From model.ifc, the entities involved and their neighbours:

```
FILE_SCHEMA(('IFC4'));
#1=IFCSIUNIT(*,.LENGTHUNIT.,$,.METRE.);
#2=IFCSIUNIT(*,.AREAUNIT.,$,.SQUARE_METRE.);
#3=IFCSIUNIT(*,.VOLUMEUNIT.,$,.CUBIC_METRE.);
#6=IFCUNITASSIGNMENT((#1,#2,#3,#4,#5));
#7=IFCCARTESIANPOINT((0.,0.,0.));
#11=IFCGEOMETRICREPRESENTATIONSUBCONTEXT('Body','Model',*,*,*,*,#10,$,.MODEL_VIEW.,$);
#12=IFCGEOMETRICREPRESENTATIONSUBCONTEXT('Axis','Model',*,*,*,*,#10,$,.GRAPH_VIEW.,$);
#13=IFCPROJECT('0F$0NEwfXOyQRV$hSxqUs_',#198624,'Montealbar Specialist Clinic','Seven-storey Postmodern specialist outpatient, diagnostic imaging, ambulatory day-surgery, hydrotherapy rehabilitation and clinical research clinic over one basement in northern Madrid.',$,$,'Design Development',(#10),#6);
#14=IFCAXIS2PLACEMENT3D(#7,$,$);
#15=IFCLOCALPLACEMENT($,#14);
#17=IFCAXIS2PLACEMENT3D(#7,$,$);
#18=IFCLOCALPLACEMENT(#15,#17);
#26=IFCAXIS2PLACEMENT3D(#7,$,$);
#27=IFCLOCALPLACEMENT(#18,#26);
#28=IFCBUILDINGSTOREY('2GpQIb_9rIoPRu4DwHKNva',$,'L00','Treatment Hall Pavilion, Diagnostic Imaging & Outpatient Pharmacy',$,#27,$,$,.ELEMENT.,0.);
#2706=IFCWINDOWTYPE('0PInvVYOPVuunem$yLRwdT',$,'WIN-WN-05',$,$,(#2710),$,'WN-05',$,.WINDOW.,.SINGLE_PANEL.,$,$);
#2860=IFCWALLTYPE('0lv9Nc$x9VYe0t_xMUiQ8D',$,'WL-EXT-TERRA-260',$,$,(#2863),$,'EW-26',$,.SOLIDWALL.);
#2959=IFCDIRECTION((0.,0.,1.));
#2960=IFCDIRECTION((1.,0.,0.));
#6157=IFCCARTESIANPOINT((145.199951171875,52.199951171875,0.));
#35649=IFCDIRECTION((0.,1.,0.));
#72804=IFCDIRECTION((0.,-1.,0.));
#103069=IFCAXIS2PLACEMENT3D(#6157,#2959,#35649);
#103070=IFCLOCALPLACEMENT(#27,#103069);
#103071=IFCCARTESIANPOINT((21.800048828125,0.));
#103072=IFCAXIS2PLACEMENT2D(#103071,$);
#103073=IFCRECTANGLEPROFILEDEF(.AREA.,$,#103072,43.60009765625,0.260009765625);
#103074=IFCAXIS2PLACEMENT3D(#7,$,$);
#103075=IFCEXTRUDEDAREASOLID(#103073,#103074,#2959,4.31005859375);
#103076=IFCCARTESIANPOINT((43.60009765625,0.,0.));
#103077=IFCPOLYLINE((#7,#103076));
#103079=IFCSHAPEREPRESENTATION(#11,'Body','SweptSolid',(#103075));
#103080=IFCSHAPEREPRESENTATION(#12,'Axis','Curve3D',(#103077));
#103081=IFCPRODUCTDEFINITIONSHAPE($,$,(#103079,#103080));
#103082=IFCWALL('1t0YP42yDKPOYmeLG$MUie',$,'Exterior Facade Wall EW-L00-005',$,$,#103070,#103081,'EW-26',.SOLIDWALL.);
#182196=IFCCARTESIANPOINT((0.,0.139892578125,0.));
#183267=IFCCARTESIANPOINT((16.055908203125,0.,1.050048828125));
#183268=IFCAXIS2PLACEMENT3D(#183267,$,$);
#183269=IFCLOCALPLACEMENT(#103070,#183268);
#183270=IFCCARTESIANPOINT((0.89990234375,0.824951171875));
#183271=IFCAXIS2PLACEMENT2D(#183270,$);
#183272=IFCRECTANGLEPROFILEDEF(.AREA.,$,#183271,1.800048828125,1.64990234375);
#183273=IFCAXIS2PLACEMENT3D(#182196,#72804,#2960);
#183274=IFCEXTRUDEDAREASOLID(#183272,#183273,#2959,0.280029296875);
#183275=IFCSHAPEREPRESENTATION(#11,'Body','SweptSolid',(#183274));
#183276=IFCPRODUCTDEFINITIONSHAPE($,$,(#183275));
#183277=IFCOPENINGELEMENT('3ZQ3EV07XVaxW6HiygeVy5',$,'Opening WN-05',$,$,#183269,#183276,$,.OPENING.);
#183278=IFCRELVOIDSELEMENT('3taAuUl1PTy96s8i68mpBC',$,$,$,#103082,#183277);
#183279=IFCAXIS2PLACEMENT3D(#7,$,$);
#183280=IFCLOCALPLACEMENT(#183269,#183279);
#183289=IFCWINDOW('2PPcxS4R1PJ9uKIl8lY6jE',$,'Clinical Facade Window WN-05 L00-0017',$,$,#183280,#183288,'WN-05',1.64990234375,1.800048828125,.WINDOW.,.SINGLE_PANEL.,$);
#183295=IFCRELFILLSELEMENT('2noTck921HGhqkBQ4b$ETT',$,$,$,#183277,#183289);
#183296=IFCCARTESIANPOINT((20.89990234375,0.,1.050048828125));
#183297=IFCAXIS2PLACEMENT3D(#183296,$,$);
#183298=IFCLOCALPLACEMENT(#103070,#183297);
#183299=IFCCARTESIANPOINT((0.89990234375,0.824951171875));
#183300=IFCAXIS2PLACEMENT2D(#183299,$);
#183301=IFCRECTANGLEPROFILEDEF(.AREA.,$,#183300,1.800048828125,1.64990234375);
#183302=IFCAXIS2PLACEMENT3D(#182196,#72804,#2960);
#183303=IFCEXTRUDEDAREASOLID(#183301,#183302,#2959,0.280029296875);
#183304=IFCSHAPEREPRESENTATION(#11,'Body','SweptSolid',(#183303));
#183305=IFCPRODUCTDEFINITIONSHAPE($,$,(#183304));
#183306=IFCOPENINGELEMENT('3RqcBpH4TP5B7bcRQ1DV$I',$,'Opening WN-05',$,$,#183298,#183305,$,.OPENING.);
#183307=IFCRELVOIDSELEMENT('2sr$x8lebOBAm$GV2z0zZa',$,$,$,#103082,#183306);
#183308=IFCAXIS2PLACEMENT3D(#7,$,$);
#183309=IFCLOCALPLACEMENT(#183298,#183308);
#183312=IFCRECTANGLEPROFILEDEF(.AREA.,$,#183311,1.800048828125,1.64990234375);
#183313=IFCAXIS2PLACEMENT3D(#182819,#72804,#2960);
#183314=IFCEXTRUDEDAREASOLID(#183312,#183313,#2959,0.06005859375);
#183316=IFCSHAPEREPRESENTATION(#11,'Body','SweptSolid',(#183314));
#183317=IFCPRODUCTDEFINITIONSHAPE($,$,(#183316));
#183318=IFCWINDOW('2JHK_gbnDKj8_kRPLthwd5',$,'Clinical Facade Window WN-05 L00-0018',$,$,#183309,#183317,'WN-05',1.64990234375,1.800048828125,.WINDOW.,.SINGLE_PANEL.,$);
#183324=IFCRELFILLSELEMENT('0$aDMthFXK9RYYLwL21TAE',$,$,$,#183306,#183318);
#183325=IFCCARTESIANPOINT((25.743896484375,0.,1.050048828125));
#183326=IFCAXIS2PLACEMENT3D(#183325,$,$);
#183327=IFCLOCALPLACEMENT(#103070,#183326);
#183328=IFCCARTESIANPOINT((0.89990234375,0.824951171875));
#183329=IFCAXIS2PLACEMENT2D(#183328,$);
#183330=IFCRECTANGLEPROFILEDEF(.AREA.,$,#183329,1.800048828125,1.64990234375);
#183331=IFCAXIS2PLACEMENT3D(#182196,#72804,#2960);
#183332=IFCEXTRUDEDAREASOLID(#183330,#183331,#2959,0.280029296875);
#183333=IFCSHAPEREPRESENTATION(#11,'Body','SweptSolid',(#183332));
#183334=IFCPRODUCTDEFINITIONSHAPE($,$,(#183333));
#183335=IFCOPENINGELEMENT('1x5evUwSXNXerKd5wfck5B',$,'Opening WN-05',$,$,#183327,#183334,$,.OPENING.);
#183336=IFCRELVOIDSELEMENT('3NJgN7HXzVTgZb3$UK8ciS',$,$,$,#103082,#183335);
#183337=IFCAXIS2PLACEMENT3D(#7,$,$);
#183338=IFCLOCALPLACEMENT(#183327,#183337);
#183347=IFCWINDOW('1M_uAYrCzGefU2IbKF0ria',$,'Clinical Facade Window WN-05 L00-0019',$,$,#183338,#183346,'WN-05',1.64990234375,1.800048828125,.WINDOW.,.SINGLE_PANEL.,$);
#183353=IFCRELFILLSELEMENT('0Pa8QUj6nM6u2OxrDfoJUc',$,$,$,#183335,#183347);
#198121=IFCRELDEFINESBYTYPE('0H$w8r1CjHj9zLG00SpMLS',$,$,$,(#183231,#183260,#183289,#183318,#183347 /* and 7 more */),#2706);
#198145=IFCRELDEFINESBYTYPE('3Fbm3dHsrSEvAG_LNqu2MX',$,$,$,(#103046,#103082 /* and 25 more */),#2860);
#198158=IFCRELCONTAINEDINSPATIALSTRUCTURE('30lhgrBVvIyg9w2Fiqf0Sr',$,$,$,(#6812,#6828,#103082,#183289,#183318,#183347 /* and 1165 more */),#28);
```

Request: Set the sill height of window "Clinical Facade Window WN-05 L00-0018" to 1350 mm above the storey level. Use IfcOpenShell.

```python
import numpy as np
import ifcopenshell
import ifcopenshell.api.geometry
import ifcopenshell.geom
import ifcopenshell.util.element
import ifcopenshell.util.placement
import ifcopenshell.util.shape
import ifcopenshell.util.unit

model = ifcopenshell.open("model.ifc")
unit_scale = ifcopenshell.util.unit.calculate_unit_scale(model)

window = model.by_guid("2JHK_gbnDKj8_kRPLthwd5")
opening = window.FillsVoids[0].RelatingOpeningElement
storey = ifcopenshell.util.element.get_container(window, ifc_class="IfcBuildingStorey")
level = ifcopenshell.util.placement.get_local_placement(storey.ObjectPlacement)[2, 3]

# The opening's origin need not be at the sill, so measure its lowest point.
shape = ifcopenshell.geom.create_shape(ifcopenshell.geom.settings(), opening)
bottom = ifcopenshell.util.shape.get_shape_bottom_elevation(shape, shape.geometry) / unit_scale
dz = level + 1.35 - bottom

shift = np.array([0.0, 0.0, dz])
# The window is placed relative to its opening, so it follows when the opening moves.
matrix = ifcopenshell.util.placement.get_local_placement(opening.ObjectPlacement)
matrix[:3, 3] += shift
ifcopenshell.api.geometry.edit_object_placement(
    model, product=opening, matrix=matrix, is_si=False, should_transform_children=True
)

print(f"moved by {dz * unit_scale:+.3f} m")

model.write("model_v2.ifc")
```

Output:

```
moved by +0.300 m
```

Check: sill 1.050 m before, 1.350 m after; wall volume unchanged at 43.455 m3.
